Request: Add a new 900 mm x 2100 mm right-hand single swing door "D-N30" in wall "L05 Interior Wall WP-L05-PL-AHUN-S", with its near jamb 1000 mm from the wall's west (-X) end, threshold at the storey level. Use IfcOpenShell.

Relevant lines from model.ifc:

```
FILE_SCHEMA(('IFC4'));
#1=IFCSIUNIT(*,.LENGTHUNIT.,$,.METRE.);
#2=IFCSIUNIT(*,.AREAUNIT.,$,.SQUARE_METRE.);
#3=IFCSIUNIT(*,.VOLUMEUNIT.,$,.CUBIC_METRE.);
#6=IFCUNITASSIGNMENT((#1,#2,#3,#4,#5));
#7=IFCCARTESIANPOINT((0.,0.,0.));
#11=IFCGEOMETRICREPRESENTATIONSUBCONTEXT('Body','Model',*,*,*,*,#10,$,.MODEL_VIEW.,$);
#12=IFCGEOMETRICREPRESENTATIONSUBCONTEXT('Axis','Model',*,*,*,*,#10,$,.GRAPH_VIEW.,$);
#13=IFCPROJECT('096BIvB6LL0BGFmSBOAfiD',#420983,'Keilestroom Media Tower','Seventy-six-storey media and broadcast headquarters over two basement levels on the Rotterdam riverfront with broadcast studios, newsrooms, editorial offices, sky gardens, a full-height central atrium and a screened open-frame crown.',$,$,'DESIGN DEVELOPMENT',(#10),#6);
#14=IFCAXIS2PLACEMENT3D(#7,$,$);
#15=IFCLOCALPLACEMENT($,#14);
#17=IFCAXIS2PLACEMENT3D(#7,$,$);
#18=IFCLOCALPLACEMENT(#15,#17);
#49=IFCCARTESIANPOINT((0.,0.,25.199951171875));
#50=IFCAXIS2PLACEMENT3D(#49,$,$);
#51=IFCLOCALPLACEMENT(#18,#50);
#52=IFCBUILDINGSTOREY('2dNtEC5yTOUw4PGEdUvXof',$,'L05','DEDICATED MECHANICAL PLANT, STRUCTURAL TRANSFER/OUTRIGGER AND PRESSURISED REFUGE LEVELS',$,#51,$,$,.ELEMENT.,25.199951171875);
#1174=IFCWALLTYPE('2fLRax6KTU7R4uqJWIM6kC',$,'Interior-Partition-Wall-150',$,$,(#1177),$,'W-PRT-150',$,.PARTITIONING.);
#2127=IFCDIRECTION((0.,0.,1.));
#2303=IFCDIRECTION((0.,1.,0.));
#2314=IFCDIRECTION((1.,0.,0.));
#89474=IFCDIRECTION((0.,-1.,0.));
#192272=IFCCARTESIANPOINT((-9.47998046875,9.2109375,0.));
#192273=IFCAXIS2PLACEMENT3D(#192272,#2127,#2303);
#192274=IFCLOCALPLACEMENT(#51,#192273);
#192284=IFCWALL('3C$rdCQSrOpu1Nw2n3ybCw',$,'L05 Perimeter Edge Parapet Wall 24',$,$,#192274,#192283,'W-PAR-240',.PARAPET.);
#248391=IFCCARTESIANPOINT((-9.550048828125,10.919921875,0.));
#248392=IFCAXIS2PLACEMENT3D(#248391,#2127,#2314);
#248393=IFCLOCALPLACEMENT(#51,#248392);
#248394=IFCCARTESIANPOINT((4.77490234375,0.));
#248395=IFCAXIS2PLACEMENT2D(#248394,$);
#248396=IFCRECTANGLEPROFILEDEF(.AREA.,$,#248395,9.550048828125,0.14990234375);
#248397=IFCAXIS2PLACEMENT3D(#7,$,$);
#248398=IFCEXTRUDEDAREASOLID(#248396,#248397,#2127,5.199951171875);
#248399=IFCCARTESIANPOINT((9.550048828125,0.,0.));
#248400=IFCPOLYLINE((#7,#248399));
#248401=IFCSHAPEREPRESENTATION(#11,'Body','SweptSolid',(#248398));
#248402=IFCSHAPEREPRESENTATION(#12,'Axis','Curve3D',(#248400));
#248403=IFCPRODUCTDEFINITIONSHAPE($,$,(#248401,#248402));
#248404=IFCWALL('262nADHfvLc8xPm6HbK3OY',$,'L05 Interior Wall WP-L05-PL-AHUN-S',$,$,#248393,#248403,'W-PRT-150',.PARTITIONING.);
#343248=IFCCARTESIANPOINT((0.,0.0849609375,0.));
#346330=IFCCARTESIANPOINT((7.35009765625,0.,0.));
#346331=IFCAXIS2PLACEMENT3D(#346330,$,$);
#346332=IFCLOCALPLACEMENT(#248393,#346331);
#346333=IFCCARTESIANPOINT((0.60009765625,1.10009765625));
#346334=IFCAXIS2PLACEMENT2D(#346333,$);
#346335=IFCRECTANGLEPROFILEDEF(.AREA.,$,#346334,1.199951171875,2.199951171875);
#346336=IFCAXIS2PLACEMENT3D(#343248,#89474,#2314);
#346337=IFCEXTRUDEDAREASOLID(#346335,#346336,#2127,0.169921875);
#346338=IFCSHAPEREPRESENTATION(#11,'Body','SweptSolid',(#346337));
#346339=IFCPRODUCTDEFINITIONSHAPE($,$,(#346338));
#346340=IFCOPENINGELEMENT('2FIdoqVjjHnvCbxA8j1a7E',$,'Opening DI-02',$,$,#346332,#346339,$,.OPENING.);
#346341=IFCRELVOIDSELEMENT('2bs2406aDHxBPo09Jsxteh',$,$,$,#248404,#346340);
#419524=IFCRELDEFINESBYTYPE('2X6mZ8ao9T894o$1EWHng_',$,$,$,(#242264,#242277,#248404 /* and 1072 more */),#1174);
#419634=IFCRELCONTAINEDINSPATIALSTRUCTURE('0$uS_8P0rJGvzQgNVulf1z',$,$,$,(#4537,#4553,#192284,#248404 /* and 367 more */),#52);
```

```python
import numpy as np
import ifcopenshell
import ifcopenshell.api.feature
import ifcopenshell.api.geometry
import ifcopenshell.api.root
import ifcopenshell.api.spatial
import ifcopenshell.geom
import ifcopenshell.util.element
import ifcopenshell.util.placement
import ifcopenshell.util.representation
import ifcopenshell.util.shape
import ifcopenshell.util.unit

model = ifcopenshell.open("model.ifc")
unit_scale = ifcopenshell.util.unit.calculate_unit_scale(model)
settings = ifcopenshell.geom.settings()


def volume(element):
    """Net volume in cubic metres, openings subtracted."""
    shape = ifcopenshell.geom.create_shape(settings, element)
    return ifcopenshell.util.shape.get_volume(shape.geometry)


wall = model.by_guid("262nADHfvLc8xPm6HbK3OY")
storey = ifcopenshell.util.element.get_container(wall, ifc_class="IfcBuildingStorey")
context = ifcopenshell.util.representation.get_context(model, "Model", "Body", "MODEL_VIEW")
before = volume(wall)

width, height, from_end, sill = 0.9, 2.1, 1, 0.0  # metres

# The wall runs along its own X axis, and the end named is its -X end.
wall_shape = ifcopenshell.geom.create_shape(settings, wall)
x, y, z = ifcopenshell.util.shape.get_vertices(wall_shape.geometry).T
start = x.min() + from_end
face, thickness = float(y.min()), float(y.max() - y.min())
wall_matrix = ifcopenshell.util.placement.get_local_placement(wall.ObjectPlacement)
level = ifcopenshell.util.placement.get_local_placement(storey.ObjectPlacement)[2, 3]


def in_wall(x, y):
    """Placement at x, y metres in the wall's axes, at sill height."""
    matrix = wall_matrix.copy()
    matrix[:, 3] = wall_matrix @ np.array([x / unit_scale, y / unit_scale, 0.0, 1.0])
    matrix[2, 3] = level + sill / unit_scale
    return matrix


# Opening: a box that overshoots both wall faces by 50 mm.
opening = ifcopenshell.api.root.create_entity(model, ifc_class="IfcOpeningElement", predefined_type="OPENING")
box = ifcopenshell.api.geometry.add_wall_representation(
    model, context=context, length=width, height=height, thickness=thickness + 0.1
)
ifcopenshell.api.geometry.assign_representation(model, product=opening, representation=box)
ifcopenshell.api.geometry.edit_object_placement(model, product=opening, matrix=in_wall(start, face - 0.05), is_si=False)
ifcopenshell.api.feature.add_feature(model, feature=opening, element=wall)

door = ifcopenshell.api.root.create_entity(model, ifc_class="IfcDoor", name="D-N30", predefined_type="DOOR")
door.OverallWidth, door.OverallHeight = width / unit_scale, height / unit_scale
door.OperationType = "SINGLE_SWING_RIGHT"
body = ifcopenshell.api.geometry.add_door_representation(
    model,
    context=context,
    overall_width=door.OverallWidth,
    overall_height=door.OverallHeight,
    operation_type="SINGLE_SWING_RIGHT",
    lining_properties={"LiningDepth": thickness / unit_scale, "ThresholdDepth": thickness / unit_scale},
)
ifcopenshell.api.geometry.assign_representation(model, product=door, representation=body)
ifcopenshell.api.spatial.assign_container(model, products=[door], relating_structure=storey)
ifcopenshell.api.feature.add_filling(model, opening=opening, element=door)

# The lining spans the wall, so the door starts at the wall face.
ifcopenshell.api.geometry.edit_object_placement(model, product=door, matrix=in_wall(start, face), is_si=False)

after = volume(wall)

print(f"wall volume {before:.3f} -> {after:.3f} m3")

model.write("model-out.ifc")
```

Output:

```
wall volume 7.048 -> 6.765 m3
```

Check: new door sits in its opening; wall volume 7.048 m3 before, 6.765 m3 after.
